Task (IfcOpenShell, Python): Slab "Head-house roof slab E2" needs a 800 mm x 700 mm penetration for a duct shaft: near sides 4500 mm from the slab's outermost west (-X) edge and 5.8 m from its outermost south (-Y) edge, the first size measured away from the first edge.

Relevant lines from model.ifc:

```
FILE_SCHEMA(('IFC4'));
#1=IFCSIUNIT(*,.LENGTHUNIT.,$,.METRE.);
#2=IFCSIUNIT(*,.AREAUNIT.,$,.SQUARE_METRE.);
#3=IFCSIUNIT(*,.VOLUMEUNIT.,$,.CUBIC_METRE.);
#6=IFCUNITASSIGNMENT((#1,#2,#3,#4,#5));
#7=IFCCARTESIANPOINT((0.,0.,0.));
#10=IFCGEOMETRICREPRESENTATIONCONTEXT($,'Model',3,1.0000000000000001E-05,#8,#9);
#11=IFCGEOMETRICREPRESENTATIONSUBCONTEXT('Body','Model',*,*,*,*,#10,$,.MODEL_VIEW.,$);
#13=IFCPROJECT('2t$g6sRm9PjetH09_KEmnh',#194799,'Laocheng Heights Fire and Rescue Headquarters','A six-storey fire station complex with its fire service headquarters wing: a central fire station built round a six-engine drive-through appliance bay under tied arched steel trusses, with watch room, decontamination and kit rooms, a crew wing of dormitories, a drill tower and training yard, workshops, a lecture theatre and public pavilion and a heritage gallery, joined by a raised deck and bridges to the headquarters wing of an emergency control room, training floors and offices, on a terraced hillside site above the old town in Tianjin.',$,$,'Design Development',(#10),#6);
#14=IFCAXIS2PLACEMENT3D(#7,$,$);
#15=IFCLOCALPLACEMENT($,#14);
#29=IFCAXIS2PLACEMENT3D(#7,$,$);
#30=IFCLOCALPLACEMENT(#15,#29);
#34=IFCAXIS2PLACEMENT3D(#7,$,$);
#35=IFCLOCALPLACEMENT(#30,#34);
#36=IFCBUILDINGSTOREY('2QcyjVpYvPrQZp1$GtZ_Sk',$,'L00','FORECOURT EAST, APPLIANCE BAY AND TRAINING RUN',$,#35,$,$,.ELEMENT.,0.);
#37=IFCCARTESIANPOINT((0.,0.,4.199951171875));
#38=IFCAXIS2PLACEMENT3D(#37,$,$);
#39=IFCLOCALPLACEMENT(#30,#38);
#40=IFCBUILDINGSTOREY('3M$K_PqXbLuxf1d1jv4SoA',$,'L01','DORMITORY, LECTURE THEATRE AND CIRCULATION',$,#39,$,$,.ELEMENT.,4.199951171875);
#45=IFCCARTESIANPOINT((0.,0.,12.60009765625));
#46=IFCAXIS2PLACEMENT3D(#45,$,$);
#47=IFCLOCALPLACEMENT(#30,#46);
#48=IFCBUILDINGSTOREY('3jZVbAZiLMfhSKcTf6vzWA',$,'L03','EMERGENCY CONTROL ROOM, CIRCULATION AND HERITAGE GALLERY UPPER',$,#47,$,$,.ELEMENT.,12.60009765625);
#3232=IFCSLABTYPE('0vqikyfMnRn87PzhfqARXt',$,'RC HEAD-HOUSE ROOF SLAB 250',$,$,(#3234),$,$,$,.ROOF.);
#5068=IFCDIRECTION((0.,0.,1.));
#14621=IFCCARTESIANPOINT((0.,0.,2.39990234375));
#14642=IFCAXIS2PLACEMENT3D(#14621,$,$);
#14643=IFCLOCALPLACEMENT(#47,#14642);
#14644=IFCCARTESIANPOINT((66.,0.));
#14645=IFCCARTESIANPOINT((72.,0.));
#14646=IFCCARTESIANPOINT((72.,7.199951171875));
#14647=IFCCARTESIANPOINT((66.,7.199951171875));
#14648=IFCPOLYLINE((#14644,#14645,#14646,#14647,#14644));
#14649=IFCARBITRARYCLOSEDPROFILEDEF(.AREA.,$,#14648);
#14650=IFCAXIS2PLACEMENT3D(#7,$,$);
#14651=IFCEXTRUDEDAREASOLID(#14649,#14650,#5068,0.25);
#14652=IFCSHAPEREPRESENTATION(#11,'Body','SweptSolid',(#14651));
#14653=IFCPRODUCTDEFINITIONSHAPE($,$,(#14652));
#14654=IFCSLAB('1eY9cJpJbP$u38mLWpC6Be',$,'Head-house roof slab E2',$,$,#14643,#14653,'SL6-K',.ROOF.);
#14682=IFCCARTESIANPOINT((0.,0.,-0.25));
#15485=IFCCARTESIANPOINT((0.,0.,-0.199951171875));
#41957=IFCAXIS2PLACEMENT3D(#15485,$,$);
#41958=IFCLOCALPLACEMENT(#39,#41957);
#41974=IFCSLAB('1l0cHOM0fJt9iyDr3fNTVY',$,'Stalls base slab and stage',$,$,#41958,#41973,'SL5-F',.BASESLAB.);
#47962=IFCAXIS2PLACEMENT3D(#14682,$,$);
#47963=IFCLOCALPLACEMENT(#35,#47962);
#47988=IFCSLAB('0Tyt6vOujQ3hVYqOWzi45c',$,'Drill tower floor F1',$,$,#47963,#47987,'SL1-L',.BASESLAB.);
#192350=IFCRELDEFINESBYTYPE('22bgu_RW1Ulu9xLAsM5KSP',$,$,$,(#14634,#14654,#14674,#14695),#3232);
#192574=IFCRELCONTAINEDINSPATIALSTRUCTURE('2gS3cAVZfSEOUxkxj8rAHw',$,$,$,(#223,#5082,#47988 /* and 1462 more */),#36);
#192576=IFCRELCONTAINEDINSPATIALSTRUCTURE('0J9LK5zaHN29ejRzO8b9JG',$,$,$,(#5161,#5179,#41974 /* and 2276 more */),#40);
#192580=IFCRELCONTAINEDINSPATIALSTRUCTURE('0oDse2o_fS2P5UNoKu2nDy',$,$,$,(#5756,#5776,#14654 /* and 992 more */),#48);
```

```python
import numpy as np
import ifcopenshell
import ifcopenshell.api.feature
import ifcopenshell.api.geometry
import ifcopenshell.api.root
import ifcopenshell.geom
import ifcopenshell.util.placement
import ifcopenshell.util.representation
import ifcopenshell.util.shape
import ifcopenshell.util.unit

model = ifcopenshell.open("model.ifc")
unit_scale = ifcopenshell.util.unit.calculate_unit_scale(model)
settings = ifcopenshell.geom.settings()


def volume(element):
    """Net volume in cubic metres, openings subtracted."""
    shape = ifcopenshell.geom.create_shape(settings, element)
    return ifcopenshell.util.shape.get_volume(shape.geometry)


slab = model.by_guid("1eY9cJpJbP$u38mLWpC6Be")
before = volume(slab)

# Extent in the slab's own axes, in metres. The edges named are its -X and -Y sides.
slab_shape = ifcopenshell.geom.create_shape(settings, slab)
vertices = ifcopenshell.util.shape.get_vertices(slab_shape.geometry)
x_min, y_min, bottom = vertices.min(axis=0)
top = vertices[:, 2].max()

opening = ifcopenshell.api.root.create_entity(model, ifc_class="IfcOpeningElement", name="Duct shaft opening", predefined_type="OPENING")
context = ifcopenshell.util.representation.get_context(model, "Model", "Body", "MODEL_VIEW")
width, depth = 0.8, 0.7
outline = [(0.0, 0.0), (width, 0.0), (width, depth), (0.0, depth), (0.0, 0.0)]
# Overshoot both faces by 50 mm so the cut is clean.
shape = ifcopenshell.api.geometry.add_slab_representation(
    model, context=context, depth=top - bottom + 0.1, polyline=outline
)
ifcopenshell.api.geometry.assign_representation(model, product=opening, representation=shape)

matrix = ifcopenshell.util.placement.get_local_placement(slab.ObjectPlacement)
matrix[:, 3] = matrix @ np.append(np.array([x_min + 4.5, y_min + 5.8, bottom - 0.05]) / unit_scale, 1.0)
ifcopenshell.api.geometry.edit_object_placement(model, product=opening, matrix=matrix, is_si=False)
ifcopenshell.api.feature.add_feature(model, feature=opening, element=slab)

after = volume(slab)

print(f"slab volume {before:.3f} -> {after:.3f} m3")

model.write("model_v2.ifc")
```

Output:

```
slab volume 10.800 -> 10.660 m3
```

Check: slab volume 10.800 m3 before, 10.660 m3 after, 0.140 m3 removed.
